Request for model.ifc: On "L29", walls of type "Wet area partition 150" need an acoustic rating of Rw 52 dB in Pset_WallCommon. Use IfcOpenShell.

First a look at what the model holds.

```python
import ifcopenshell
import ifcopenshell.util.element

model = ifcopenshell.open("model.ifc")
print(model.schema)
storey = next(s for s in model.by_type("IfcBuildingStorey") if s.Name == "L29")
walls = [e for e in ifcopenshell.util.element.get_decomposition(storey) if e.is_a("IfcWall")]
seen = {}
for e in walls:
    element_type = ifcopenshell.util.element.get_type(e)
    key = (element_type.Name if element_type != e and element_type else None, ifcopenshell.util.element.get_pset(e, "Pset_WallCommon", "AcousticRating"))
    seen[key] = seen.get(key, 0) + 1
for (name, value), count in sorted(seen.items(), key=str):
    print(count, "x", name, "|", value)
```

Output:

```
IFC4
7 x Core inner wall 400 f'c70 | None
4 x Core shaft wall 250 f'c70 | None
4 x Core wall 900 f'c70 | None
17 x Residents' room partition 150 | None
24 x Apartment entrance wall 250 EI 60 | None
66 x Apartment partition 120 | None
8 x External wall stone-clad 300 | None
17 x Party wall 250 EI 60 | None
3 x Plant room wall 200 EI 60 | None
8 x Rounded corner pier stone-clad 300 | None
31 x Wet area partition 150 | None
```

```python
import ifcopenshell
import ifcopenshell.api.pset
import ifcopenshell.util.element

model = ifcopenshell.open("model.ifc")

storey = next(s for s in model.by_type("IfcBuildingStorey") if s.Name == "L29")
walls = [e for e in ifcopenshell.util.element.get_decomposition(storey) if e.is_a("IfcWall")]

count = 0
for e in walls:
    element_type = ifcopenshell.util.element.get_type(e)
    if element_type in (None, e) or element_type.Name != "Wet area partition 150":
        continue
    found = ifcopenshell.util.element.get_pset(e, "Pset_WallCommon", should_inherit=False)
    if found:
        pset = model.by_id(found["id"])
        if len(ifcopenshell.util.element.get_elements_by_pset(pset)) > 1:
            pset = ifcopenshell.api.pset.unshare_pset(model, products=[e], pset=pset)[0]
    else:
        pset = ifcopenshell.api.pset.add_pset(model, product=e, name="Pset_WallCommon")
    ifcopenshell.api.pset.edit_pset(model, pset=pset, properties={"AcousticRating": "Rw 52 dB"})
    count += 1

print(count, "walls updated")

model.write("model_v2.ifc")
```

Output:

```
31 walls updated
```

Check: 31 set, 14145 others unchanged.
